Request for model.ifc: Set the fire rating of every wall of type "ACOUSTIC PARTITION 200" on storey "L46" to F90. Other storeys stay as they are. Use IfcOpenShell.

First a look at what the model holds.

```python
import ifcopenshell
import ifcopenshell.util.element

model = ifcopenshell.open("model.ifc")
print(model.schema)
storey = next(s for s in model.by_type("IfcBuildingStorey") if s.Name == "L46")
walls = [e for e in ifcopenshell.util.element.get_decomposition(storey) if e.is_a("IfcWall")]
seen = {}
for e in walls:
    element_type = ifcopenshell.util.element.get_type(e)
    key = (element_type.Name if element_type != e and element_type else None, ifcopenshell.util.element.get_pset(e, "Pset_WallCommon", "FireRating"))
    seen[key] = seen.get(key, 0) + 1
for (name, value), count in sorted(seen.items(), key=str):
    print(count, "x", name, "|", value)
```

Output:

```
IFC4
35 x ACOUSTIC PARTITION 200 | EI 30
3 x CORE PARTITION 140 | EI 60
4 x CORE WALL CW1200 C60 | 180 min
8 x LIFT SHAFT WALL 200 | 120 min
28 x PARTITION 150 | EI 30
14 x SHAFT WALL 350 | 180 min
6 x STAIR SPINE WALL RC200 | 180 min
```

```python
import ifcopenshell
import ifcopenshell.api.pset
import ifcopenshell.util.element

model = ifcopenshell.open("model.ifc")

storey = next(s for s in model.by_type("IfcBuildingStorey") if s.Name == "L46")
walls = [e for e in ifcopenshell.util.element.get_decomposition(storey) if e.is_a("IfcWall")]

count = 0
for e in walls:
    element_type = ifcopenshell.util.element.get_type(e)
    if element_type in (None, e) or element_type.Name != "ACOUSTIC PARTITION 200":
        continue
    found = ifcopenshell.util.element.get_pset(e, "Pset_WallCommon", should_inherit=False)
    if found:
        pset = model.by_id(found["id"])
        if len(ifcopenshell.util.element.get_elements_by_pset(pset)) > 1:
            pset = ifcopenshell.api.pset.unshare_pset(model, products=[e], pset=pset)[0]
    else:
        pset = ifcopenshell.api.pset.add_pset(model, product=e, name="Pset_WallCommon")
    ifcopenshell.api.pset.edit_pset(model, pset=pset, properties={"FireRating": "F90"})
    count += 1

print(count, "walls updated")

model.write("model_updated.ifc")
```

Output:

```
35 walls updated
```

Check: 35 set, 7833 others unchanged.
